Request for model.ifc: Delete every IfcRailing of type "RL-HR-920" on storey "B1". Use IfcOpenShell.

First a look at what the model holds.

```python
import ifcopenshell
import ifcopenshell.util.element

model = ifcopenshell.open("model.ifc")
print(model.schema)
storey = next(s for s in model.by_type("IfcBuildingStorey") if s.Name == "B1")
railings = [e for e in ifcopenshell.util.element.get_decomposition(storey) if e.is_a("IfcRailing")]
seen = {}
for e in railings:
    element_type = ifcopenshell.util.element.get_type(e)
    name = element_type.Name if element_type not in (None, e) else None
    seen[name] = seen.get(name, 0) + 1
for name, count in sorted(seen.items(), key=str):
    print(count, "x", name)
```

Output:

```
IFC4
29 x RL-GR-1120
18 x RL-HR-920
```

```python
import ifcopenshell
import ifcopenshell.api.root
import ifcopenshell.util.element

model = ifcopenshell.open("model.ifc")

storey = next(s for s in model.by_type("IfcBuildingStorey") if s.Name == "B1")
railings = [e for e in ifcopenshell.util.element.get_decomposition(storey) if e.is_a("IfcRailing")]
targets = [e for e in railings if (t := ifcopenshell.util.element.get_type(e)) not in (None, e) and t.Name == "RL-HR-920"]

for e in targets:
    ifcopenshell.api.root.remove_product(model, product=e)
print(len(targets), "removed")

model.write("model_edited.ifc")
```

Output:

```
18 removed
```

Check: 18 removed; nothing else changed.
